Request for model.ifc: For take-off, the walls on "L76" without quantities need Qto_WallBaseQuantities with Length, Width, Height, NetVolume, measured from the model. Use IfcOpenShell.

First a look at what the model holds.

```python
import ifcopenshell
import ifcopenshell.util.element
import ifcopenshell.util.unit

model = ifcopenshell.open("model.ifc")
print(model.schema)
for unit_type in ("LENGTHUNIT", "AREAUNIT", "VOLUMEUNIT"):
    print(unit_type, ifcopenshell.util.unit.calculate_unit_scale(model, unit_type))
storey = next(s for s in model.by_type("IfcBuildingStorey") if s.Name == "L76")
walls = [e for e in ifcopenshell.util.element.get_decomposition(storey) if e.is_a("IfcWall")]
for e in sorted(walls, key=lambda e: e.id()):
    print(e.id(), e.is_a(), e.Name, list(ifcopenshell.util.element.get_psets(e, qtos_only=True)), sep=" | ")
```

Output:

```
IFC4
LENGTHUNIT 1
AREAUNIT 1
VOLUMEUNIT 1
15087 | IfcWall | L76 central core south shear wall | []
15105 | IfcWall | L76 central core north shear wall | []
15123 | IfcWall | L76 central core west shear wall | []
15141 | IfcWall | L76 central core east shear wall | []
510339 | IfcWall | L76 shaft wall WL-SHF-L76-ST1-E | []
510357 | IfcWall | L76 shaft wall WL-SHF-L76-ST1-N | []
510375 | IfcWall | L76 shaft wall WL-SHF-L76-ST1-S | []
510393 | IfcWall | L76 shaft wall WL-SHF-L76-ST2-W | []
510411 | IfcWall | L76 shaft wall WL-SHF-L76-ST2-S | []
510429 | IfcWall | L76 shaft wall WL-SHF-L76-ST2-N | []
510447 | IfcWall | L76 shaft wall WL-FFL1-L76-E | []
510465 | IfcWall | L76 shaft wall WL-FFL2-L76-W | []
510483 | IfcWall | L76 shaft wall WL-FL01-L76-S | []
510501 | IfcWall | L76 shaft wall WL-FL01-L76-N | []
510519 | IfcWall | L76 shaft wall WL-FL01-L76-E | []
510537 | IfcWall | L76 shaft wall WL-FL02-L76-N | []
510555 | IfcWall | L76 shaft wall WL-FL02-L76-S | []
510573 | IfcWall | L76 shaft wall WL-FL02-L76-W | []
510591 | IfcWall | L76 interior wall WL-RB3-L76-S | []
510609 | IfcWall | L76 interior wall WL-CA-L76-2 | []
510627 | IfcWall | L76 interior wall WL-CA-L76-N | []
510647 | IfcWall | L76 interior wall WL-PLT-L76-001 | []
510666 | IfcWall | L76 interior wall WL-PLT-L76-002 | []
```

```python
import ifcopenshell
import ifcopenshell.api.pset
import ifcopenshell.geom
import ifcopenshell.util.element
import ifcopenshell.util.shape
import ifcopenshell.util.unit

model = ifcopenshell.open("model.ifc")
unit_scale = ifcopenshell.util.unit.calculate_unit_scale(model)
volume_scale = ifcopenshell.util.unit.calculate_unit_scale(model, "VOLUMEUNIT")
settings = ifcopenshell.geom.settings()

storey = next(s for s in model.by_type("IfcBuildingStorey") if s.Name == "L76")
walls = [e for e in ifcopenshell.util.element.get_decomposition(storey) if e.is_a("IfcWall")]

for e in sorted(walls, key=lambda e: e.id()):
    if ifcopenshell.util.element.get_psets(e, qtos_only=True, should_inherit=False):
        continue
    # Geometry comes back in metres, in the element's own axes.
    shape = ifcopenshell.geom.create_shape(settings, e)
    values = {
        "Length": ifcopenshell.util.shape.get_x(shape.geometry) / unit_scale,
        "Width": ifcopenshell.util.shape.get_y(shape.geometry) / unit_scale,
        "Height": ifcopenshell.util.shape.get_z(shape.geometry) / unit_scale,
        "NetVolume": ifcopenshell.util.shape.get_volume(shape.geometry) / volume_scale,
    }
    qto = ifcopenshell.api.pset.add_qto(model, product=e, name="Qto_WallBaseQuantities")
    ifcopenshell.api.pset.edit_qto(model, qto=qto, properties=values)
    print(e.id(), {k: round(v, 3) for k, v in values.items()})

model.write("model_v2.ifc")
```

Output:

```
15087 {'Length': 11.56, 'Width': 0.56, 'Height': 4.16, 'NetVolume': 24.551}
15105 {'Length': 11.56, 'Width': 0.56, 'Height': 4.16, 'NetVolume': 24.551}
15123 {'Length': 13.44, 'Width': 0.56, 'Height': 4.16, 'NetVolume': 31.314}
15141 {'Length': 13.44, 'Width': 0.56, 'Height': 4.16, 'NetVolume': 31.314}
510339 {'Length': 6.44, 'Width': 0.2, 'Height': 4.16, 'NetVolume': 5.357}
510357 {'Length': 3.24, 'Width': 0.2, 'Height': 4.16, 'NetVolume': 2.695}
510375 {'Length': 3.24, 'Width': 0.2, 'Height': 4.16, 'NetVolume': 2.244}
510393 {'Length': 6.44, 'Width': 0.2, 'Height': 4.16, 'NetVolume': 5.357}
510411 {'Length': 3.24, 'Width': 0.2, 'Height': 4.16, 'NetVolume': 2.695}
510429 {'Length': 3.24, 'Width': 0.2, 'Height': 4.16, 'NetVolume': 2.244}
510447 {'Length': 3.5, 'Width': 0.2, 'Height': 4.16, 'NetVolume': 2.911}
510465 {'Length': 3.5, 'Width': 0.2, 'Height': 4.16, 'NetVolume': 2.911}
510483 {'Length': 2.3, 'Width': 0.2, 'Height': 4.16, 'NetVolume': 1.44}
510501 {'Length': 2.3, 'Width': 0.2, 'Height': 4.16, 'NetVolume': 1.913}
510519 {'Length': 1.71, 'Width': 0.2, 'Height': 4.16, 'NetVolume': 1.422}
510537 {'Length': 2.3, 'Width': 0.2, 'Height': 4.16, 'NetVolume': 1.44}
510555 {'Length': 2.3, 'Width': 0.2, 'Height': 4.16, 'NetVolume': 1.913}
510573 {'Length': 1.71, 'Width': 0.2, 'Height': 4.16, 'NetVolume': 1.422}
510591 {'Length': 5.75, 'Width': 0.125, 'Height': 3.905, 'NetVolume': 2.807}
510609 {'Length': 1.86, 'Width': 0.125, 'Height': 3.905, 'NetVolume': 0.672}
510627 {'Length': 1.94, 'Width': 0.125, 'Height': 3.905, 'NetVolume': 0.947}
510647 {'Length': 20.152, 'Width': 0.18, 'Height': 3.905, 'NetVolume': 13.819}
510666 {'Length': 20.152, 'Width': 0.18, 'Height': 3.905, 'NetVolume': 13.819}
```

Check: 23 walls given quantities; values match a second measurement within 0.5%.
